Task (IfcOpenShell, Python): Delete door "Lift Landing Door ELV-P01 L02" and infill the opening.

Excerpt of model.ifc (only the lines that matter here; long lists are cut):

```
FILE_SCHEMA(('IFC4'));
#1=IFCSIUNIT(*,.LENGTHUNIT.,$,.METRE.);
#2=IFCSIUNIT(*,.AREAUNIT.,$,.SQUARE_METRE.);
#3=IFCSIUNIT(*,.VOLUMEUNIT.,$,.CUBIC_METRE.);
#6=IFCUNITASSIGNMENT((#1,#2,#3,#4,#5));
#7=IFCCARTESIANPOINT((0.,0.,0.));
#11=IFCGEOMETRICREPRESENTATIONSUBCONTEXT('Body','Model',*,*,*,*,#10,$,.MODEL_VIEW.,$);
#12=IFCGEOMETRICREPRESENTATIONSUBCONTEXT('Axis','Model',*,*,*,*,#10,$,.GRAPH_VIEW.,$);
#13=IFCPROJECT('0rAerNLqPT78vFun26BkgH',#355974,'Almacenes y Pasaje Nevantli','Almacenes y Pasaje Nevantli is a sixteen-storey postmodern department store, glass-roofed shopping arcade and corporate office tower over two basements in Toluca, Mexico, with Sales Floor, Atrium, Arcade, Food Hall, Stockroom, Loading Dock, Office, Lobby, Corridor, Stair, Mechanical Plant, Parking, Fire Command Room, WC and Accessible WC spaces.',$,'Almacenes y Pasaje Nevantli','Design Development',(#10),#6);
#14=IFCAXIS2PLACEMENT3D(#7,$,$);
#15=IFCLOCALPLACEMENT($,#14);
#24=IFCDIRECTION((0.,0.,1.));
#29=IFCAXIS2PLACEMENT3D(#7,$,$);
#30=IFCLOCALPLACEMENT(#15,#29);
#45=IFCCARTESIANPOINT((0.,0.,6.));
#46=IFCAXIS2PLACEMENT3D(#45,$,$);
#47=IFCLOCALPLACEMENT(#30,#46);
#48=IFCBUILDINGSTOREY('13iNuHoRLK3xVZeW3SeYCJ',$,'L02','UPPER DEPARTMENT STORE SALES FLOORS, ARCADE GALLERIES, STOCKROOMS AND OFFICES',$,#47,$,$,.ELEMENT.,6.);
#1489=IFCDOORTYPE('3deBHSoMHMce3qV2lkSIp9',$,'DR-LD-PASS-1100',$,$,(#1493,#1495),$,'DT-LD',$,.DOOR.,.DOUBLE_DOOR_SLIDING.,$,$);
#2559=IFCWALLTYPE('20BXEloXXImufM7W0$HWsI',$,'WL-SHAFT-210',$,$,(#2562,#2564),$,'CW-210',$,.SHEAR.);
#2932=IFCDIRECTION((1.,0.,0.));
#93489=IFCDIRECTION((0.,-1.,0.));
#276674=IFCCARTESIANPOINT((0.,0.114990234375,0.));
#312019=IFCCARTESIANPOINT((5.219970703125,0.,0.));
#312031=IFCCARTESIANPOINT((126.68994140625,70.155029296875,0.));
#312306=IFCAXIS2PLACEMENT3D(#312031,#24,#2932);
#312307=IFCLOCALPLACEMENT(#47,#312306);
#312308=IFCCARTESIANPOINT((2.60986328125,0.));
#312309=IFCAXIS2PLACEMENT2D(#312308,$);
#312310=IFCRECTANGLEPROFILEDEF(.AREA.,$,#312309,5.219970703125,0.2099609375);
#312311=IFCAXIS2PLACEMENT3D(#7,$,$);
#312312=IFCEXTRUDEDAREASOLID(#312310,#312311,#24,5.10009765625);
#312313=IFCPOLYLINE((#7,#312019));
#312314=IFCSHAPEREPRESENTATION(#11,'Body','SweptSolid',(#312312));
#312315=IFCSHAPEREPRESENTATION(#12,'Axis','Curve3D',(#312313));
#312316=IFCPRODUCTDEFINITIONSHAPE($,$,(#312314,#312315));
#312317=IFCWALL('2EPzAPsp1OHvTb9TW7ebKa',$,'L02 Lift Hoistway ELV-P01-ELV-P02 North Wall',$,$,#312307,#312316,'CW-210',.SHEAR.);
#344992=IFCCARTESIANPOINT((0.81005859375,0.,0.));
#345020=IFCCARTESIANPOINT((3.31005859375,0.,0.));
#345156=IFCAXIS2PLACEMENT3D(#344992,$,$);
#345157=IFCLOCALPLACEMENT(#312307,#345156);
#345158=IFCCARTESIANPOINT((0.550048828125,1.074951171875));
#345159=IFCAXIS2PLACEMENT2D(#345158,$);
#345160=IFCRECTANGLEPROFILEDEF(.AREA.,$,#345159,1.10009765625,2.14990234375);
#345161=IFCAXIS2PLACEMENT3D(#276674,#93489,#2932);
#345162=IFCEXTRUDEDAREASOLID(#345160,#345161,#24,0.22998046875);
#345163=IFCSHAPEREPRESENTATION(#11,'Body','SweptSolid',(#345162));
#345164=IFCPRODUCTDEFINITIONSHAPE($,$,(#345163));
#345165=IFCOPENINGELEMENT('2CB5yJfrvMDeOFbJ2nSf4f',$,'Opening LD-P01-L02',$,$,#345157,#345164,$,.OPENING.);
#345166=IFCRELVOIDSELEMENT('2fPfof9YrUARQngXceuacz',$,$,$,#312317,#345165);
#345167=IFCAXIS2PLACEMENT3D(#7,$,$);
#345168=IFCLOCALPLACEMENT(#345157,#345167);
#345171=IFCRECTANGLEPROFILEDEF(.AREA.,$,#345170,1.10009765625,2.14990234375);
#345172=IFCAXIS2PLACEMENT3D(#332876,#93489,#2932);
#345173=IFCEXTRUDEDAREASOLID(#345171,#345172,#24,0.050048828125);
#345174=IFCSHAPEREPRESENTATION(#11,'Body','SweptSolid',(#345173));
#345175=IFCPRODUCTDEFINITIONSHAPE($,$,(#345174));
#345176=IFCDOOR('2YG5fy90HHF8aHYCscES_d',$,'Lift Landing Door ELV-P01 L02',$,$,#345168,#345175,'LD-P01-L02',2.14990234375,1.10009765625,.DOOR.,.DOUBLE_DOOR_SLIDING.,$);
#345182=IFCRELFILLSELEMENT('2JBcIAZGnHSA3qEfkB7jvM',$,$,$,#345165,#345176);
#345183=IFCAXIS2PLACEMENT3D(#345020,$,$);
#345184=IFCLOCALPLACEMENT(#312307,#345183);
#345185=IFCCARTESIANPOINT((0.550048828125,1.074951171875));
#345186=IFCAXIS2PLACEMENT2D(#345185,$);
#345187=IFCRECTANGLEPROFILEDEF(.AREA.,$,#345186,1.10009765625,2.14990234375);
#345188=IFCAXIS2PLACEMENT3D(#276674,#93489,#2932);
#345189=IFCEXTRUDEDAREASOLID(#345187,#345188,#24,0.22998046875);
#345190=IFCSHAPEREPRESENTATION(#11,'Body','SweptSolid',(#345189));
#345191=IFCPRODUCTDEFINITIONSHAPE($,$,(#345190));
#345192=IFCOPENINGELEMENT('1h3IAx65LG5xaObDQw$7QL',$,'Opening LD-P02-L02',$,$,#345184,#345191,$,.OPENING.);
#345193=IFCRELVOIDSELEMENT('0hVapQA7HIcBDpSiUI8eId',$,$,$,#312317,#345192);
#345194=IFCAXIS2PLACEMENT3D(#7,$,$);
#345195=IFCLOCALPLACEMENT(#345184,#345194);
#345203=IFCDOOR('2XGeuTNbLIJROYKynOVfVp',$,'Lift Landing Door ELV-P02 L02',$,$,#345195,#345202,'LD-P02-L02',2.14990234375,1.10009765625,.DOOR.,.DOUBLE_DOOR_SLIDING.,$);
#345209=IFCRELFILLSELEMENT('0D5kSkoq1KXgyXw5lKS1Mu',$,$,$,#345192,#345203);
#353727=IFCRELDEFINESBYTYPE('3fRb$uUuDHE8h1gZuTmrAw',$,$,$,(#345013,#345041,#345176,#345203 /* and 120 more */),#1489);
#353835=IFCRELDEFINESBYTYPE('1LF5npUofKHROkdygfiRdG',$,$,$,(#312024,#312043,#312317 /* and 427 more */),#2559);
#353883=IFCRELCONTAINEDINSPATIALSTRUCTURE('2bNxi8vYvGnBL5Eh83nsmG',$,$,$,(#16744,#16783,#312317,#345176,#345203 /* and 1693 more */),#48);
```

```python
import ifcopenshell
import ifcopenshell.api.feature
import ifcopenshell.api.root
import ifcopenshell.geom
import ifcopenshell.util.shape

model = ifcopenshell.open("model.ifc")
settings = ifcopenshell.geom.settings()


def volume(element):
    """Net volume in cubic metres, openings subtracted."""
    shape = ifcopenshell.geom.create_shape(settings, element)
    return ifcopenshell.util.shape.get_volume(shape.geometry)


door = model.by_guid("2YG5fy90HHF8aHYCscES_d")
opening = door.FillsVoids[0].RelatingOpeningElement
wall = opening.VoidsElements[0].RelatingBuildingElement
before = volume(wall)

ifcopenshell.api.root.remove_product(model, product=door)
ifcopenshell.api.feature.remove_feature(model, feature=opening)

after = volume(wall)

print(f"wall volume {before:.3f} -> {after:.3f} m3")

model.write("model_rev.ifc")
```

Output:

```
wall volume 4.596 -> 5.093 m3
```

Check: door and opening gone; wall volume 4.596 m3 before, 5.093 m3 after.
